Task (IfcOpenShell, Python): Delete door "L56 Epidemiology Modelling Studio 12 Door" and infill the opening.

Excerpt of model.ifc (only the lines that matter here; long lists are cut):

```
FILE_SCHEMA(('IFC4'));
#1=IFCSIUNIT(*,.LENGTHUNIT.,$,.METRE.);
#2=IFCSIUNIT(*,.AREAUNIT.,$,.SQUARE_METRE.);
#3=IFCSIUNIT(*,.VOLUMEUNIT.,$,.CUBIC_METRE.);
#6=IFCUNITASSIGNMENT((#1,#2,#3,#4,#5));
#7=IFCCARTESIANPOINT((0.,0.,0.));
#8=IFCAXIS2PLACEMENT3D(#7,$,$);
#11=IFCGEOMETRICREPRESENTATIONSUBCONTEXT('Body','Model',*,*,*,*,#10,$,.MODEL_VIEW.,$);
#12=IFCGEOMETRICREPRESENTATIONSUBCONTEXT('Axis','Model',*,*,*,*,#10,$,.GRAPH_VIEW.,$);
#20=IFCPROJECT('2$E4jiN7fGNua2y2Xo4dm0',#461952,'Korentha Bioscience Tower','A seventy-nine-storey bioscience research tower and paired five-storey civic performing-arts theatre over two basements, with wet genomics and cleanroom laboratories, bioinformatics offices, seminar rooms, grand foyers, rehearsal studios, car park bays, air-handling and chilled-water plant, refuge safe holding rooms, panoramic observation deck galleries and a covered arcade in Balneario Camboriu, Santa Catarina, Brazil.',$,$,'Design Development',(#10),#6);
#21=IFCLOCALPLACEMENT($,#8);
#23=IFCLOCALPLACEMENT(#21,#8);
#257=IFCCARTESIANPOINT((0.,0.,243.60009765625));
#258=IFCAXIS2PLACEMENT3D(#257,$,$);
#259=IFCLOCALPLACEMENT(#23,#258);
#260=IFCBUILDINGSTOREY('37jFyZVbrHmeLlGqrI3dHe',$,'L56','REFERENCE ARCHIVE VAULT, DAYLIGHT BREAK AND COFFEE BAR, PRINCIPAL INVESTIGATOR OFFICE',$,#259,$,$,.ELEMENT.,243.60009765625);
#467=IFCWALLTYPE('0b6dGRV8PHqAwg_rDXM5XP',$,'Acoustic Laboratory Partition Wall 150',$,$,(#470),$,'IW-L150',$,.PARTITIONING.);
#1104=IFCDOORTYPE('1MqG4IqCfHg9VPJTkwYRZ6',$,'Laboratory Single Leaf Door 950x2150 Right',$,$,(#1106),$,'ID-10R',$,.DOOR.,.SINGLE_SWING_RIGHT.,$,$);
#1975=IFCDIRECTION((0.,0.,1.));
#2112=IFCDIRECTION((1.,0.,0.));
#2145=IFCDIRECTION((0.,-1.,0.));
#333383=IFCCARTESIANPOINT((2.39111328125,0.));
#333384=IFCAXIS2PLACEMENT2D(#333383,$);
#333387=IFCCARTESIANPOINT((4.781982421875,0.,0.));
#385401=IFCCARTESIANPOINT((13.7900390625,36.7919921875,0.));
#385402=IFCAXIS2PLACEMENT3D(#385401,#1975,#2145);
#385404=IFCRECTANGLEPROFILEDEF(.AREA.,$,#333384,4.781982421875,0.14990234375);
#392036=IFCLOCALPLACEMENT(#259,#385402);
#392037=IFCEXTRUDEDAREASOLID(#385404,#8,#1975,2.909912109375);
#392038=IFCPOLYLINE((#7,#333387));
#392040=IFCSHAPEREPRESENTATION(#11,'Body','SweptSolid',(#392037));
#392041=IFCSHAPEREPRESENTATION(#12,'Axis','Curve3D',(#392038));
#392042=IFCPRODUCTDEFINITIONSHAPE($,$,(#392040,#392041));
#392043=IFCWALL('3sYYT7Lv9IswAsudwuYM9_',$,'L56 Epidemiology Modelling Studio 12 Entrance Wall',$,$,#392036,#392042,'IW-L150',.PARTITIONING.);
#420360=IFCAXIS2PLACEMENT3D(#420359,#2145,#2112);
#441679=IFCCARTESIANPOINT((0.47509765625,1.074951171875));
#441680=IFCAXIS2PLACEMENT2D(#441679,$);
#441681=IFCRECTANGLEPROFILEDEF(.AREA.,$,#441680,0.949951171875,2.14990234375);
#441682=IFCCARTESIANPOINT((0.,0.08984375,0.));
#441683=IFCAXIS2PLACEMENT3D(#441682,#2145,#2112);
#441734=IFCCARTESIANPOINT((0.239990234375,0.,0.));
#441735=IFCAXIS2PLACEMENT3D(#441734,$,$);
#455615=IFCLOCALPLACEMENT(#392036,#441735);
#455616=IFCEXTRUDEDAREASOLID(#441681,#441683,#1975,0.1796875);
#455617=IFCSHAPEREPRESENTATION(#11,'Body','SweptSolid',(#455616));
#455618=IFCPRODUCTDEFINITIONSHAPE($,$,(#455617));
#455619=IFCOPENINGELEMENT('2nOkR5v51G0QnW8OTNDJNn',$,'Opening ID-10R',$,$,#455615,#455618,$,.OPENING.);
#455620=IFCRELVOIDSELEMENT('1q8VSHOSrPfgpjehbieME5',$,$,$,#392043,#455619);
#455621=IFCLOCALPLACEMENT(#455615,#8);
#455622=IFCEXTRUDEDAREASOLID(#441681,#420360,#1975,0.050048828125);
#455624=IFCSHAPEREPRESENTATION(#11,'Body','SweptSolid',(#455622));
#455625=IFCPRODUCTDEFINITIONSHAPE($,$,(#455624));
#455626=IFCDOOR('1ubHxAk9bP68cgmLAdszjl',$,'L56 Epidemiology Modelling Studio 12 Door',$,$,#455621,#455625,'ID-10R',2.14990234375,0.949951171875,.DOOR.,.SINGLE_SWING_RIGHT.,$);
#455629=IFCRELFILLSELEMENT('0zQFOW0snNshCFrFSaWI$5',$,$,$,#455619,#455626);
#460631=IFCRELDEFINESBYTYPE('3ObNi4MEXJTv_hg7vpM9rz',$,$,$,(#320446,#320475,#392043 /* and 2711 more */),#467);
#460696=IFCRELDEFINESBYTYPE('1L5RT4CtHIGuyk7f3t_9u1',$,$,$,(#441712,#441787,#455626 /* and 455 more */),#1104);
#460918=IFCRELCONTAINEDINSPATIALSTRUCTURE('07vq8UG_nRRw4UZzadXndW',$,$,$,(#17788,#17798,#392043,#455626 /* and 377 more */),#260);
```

```python
import ifcopenshell
import ifcopenshell.api.feature
import ifcopenshell.api.root
import ifcopenshell.geom
import ifcopenshell.util.shape

model = ifcopenshell.open("model.ifc")
settings = ifcopenshell.geom.settings()


def volume(element):
    """Net volume in cubic metres, openings subtracted."""
    shape = ifcopenshell.geom.create_shape(settings, element)
    return ifcopenshell.util.shape.get_volume(shape.geometry)


door = model.by_guid("1ubHxAk9bP68cgmLAdszjl")
opening = door.FillsVoids[0].RelatingOpeningElement
wall = opening.VoidsElements[0].RelatingBuildingElement
before = volume(wall)

ifcopenshell.api.root.remove_product(model, product=door)
ifcopenshell.api.feature.remove_feature(model, feature=opening)

after = volume(wall)

print(f"wall volume {before:.3f} -> {after:.3f} m3")

model.write("model_rev.ifc")
```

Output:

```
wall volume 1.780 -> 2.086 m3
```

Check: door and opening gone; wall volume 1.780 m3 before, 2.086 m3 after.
